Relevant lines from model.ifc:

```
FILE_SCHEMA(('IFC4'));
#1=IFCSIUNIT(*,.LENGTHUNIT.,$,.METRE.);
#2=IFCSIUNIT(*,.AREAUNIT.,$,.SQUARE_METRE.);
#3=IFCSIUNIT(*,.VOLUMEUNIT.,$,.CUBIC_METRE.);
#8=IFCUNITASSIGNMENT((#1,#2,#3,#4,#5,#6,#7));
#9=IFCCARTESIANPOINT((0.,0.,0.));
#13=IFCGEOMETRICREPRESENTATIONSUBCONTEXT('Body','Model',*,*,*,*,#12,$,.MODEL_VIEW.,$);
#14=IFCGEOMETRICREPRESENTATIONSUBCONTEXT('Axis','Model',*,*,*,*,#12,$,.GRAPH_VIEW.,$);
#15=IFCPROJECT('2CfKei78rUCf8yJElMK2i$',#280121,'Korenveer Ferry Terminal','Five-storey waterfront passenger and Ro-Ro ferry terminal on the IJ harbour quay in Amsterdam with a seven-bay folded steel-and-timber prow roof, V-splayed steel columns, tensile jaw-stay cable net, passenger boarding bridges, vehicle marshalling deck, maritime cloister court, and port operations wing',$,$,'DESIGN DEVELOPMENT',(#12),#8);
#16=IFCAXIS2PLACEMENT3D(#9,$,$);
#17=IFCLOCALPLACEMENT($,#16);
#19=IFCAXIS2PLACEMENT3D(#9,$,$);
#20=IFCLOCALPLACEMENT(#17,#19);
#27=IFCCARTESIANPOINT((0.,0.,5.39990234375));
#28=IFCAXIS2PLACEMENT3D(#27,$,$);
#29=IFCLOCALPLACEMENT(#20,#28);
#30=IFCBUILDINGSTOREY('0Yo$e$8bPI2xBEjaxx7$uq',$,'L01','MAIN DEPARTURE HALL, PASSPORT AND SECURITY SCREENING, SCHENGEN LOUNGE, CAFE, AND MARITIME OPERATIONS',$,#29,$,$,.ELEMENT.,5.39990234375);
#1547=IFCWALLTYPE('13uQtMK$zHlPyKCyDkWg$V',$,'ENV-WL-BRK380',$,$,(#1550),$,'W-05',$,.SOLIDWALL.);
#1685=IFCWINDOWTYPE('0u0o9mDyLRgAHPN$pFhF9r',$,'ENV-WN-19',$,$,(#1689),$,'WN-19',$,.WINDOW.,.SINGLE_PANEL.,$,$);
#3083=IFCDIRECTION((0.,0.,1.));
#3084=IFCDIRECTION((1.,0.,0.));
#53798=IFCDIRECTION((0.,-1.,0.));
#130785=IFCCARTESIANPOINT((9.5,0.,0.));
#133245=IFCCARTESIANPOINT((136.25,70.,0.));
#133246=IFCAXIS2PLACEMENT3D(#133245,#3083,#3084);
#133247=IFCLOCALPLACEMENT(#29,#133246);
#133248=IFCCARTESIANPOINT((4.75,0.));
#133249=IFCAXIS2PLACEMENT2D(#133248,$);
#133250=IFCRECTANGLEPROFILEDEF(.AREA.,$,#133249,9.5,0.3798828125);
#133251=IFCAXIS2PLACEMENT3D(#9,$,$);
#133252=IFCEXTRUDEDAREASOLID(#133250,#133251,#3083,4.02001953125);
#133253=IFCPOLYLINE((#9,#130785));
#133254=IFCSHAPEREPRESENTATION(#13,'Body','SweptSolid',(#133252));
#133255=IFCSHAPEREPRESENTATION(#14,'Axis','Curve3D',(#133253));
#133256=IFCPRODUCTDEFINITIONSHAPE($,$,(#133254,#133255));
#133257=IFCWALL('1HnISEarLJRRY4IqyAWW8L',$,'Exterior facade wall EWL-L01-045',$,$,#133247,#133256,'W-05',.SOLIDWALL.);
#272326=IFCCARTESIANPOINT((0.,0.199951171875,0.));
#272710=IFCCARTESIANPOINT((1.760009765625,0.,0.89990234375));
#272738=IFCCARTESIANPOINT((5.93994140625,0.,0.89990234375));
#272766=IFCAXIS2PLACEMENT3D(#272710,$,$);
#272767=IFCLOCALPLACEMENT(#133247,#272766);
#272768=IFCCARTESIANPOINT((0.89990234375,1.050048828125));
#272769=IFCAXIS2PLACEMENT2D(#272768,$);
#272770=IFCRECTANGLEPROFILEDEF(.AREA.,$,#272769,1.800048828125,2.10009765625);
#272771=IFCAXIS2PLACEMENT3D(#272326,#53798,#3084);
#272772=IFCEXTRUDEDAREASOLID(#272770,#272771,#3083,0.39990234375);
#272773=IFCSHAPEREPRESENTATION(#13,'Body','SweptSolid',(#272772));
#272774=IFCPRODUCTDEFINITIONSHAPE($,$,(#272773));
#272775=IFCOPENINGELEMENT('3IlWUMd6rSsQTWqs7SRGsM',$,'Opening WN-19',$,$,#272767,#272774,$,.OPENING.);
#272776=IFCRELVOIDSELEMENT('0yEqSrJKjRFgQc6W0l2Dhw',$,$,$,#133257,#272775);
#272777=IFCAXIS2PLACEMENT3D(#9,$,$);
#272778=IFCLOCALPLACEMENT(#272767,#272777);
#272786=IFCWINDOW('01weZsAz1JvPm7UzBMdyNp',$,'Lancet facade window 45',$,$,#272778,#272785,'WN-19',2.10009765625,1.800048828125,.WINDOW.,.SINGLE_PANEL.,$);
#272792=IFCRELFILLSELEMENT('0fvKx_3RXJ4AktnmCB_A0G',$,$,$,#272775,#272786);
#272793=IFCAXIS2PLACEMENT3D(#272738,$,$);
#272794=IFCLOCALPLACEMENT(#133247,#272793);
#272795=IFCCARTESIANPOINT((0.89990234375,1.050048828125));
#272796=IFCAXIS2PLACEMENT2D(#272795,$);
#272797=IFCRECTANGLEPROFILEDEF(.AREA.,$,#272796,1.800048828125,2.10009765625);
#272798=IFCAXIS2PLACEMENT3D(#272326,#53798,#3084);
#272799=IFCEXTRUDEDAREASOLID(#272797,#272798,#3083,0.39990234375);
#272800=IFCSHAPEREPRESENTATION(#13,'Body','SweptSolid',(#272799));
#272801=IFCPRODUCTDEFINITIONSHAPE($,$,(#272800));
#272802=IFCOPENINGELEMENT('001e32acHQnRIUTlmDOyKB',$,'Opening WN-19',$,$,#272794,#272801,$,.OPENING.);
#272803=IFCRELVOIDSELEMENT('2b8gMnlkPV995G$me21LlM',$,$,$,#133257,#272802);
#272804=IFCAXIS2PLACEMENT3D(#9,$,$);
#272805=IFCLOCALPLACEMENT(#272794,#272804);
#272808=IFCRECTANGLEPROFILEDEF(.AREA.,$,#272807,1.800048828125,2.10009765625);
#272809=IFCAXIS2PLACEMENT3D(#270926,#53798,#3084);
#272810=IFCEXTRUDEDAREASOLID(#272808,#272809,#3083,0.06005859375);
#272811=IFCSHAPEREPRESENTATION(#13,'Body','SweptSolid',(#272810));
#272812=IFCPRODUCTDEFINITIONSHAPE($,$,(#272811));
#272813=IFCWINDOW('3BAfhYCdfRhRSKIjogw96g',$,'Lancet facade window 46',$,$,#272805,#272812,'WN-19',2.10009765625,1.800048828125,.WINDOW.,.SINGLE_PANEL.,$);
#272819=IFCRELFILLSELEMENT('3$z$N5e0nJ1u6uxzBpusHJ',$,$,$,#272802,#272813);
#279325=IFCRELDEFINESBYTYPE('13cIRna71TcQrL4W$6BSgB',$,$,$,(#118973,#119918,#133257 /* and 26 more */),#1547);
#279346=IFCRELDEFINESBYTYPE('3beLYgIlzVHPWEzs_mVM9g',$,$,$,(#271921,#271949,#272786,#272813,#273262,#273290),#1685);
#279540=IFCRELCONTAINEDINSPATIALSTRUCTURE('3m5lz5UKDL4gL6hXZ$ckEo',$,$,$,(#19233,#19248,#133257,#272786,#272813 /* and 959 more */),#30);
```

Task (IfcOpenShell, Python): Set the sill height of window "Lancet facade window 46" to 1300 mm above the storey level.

```python
import numpy as np
import ifcopenshell
import ifcopenshell.api.geometry
import ifcopenshell.geom
import ifcopenshell.util.element
import ifcopenshell.util.placement
import ifcopenshell.util.shape
import ifcopenshell.util.unit

model = ifcopenshell.open("model.ifc")
unit_scale = ifcopenshell.util.unit.calculate_unit_scale(model)

window = model.by_guid("3BAfhYCdfRhRSKIjogw96g")
opening = window.FillsVoids[0].RelatingOpeningElement
storey = ifcopenshell.util.element.get_container(window, ifc_class="IfcBuildingStorey")
level = ifcopenshell.util.placement.get_local_placement(storey.ObjectPlacement)[2, 3]

# The opening's origin need not be at the sill, so measure its lowest point.
shape = ifcopenshell.geom.create_shape(ifcopenshell.geom.settings(), opening)
bottom = ifcopenshell.util.shape.get_shape_bottom_elevation(shape, shape.geometry) / unit_scale
dz = level + 1.3 - bottom

shift = np.array([0.0, 0.0, dz])
# The window is placed relative to its opening, so it follows when the opening moves.
matrix = ifcopenshell.util.placement.get_local_placement(opening.ObjectPlacement)
matrix[:3, 3] += shift
ifcopenshell.api.geometry.edit_object_placement(
    model, product=opening, matrix=matrix, is_si=False, should_transform_children=True
)

print(f"moved by {dz * unit_scale:+.3f} m")

model.write("model_v2.ifc")
```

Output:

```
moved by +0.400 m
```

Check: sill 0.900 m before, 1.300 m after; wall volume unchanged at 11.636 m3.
